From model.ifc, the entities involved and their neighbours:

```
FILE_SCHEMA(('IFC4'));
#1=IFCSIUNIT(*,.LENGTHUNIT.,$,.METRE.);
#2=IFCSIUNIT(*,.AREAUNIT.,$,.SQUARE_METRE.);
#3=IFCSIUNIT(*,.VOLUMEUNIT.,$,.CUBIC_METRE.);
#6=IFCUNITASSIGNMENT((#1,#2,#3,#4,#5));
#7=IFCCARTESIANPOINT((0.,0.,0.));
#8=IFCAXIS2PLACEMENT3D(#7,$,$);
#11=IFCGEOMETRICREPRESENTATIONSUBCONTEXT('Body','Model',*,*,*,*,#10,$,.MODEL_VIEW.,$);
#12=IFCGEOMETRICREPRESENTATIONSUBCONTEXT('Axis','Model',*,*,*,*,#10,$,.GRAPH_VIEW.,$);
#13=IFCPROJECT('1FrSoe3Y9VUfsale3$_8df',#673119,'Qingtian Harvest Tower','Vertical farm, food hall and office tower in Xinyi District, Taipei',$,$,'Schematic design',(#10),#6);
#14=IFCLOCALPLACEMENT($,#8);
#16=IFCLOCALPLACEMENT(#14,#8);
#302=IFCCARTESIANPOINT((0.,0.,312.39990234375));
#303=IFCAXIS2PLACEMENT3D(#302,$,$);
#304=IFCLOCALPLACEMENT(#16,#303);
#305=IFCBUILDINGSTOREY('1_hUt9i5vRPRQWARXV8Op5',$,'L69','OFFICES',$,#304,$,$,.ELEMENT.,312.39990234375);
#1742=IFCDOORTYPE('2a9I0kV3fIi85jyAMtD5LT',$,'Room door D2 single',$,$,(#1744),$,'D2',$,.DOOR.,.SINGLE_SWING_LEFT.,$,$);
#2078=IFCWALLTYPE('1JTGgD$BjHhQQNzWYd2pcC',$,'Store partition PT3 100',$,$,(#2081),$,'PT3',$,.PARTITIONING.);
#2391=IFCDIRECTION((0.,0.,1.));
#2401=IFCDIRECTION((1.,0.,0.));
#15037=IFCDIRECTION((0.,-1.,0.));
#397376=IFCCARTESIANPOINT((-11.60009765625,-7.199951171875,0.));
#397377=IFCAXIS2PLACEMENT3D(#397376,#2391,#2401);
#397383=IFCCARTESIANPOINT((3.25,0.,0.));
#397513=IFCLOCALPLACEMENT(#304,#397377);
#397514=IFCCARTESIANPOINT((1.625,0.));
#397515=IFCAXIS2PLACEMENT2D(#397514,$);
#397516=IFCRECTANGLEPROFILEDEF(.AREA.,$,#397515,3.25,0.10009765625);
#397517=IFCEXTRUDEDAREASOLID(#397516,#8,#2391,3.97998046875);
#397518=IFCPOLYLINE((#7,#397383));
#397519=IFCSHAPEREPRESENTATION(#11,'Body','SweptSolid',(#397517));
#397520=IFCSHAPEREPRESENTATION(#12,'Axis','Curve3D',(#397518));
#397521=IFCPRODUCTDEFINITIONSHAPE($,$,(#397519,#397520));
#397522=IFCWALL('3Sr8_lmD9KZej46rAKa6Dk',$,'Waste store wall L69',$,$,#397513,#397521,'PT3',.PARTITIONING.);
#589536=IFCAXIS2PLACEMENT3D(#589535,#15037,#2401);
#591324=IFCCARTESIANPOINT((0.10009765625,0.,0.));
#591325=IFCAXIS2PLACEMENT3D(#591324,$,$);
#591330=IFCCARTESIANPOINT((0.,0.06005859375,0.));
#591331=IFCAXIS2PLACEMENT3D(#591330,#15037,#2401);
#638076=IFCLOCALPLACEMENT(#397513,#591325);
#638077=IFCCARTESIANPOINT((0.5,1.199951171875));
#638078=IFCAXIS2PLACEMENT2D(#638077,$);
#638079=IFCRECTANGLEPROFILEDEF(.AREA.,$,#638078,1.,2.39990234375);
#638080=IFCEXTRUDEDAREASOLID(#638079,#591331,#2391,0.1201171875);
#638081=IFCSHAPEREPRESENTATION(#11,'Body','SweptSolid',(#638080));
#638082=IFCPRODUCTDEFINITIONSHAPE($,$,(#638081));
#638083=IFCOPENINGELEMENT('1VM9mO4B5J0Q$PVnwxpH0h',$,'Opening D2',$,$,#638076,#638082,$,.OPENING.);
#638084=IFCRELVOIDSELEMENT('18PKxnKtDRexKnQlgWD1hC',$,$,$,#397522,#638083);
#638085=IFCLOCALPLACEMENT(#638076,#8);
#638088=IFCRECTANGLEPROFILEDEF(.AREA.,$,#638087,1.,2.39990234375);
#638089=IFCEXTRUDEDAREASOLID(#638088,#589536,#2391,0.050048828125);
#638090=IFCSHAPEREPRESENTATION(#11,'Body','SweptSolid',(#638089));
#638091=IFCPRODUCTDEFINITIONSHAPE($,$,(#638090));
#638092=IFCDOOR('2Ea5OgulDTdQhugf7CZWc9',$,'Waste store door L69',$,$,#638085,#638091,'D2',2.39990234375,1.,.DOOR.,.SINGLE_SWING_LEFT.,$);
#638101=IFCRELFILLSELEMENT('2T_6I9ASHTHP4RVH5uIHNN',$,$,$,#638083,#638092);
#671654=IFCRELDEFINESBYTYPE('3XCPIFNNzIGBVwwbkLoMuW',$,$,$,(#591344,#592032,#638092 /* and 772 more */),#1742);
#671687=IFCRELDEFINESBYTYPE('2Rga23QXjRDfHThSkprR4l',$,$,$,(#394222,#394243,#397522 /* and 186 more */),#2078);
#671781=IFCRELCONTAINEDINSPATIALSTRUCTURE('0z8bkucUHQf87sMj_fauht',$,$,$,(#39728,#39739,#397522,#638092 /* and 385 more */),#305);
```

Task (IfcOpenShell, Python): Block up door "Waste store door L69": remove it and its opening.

```python
import ifcopenshell
import ifcopenshell.api.feature
import ifcopenshell.api.root
import ifcopenshell.geom
import ifcopenshell.util.shape

model = ifcopenshell.open("model.ifc")
settings = ifcopenshell.geom.settings()


def volume(element):
    """Net volume in cubic metres, openings subtracted."""
    shape = ifcopenshell.geom.create_shape(settings, element)
    return ifcopenshell.util.shape.get_volume(shape.geometry)


door = model.by_id(638092)
opening = door.FillsVoids[0].RelatingOpeningElement
wall = opening.VoidsElements[0].RelatingBuildingElement
before = volume(wall)

ifcopenshell.api.root.remove_product(model, product=door)
ifcopenshell.api.feature.remove_feature(model, feature=opening)

after = volume(wall)

print(f"wall volume {before:.3f} -> {after:.3f} m3")

model.write("model_rev.ifc")
```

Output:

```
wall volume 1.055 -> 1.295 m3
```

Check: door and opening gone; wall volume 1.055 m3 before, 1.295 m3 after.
